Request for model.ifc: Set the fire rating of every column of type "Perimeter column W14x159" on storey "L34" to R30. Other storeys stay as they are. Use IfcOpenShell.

First a look at what the model holds.

```python
import ifcopenshell
import ifcopenshell.util.element

model = ifcopenshell.open("model.ifc")
print(model.schema)
storey = next(s for s in model.by_type("IfcBuildingStorey") if s.Name == "L34")
columns = [e for e in ifcopenshell.util.element.get_decomposition(storey) if e.is_a("IfcColumn")]
seen = {}
for e in columns:
    element_type = ifcopenshell.util.element.get_type(e)
    key = (element_type.Name if element_type != e and element_type else None, ifcopenshell.util.element.get_pset(e, "Pset_ColumnCommon", "FireRating"))
    seen[key] = seen.get(key, 0) + 1
for (name, value), count in sorted(seen.items(), key=str):
    print(count, "x", name, "|", value)
```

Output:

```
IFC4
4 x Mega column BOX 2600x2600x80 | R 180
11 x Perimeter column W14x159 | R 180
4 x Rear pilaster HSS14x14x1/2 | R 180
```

```python
import ifcopenshell
import ifcopenshell.api.pset
import ifcopenshell.util.element

model = ifcopenshell.open("model.ifc")

storey = next(s for s in model.by_type("IfcBuildingStorey") if s.Name == "L34")
columns = [e for e in ifcopenshell.util.element.get_decomposition(storey) if e.is_a("IfcColumn")]

count = 0
for e in columns:
    element_type = ifcopenshell.util.element.get_type(e)
    if element_type in (None, e) or element_type.Name != "Perimeter column W14x159":
        continue
    found = ifcopenshell.util.element.get_pset(e, "Pset_ColumnCommon", should_inherit=False)
    if found:
        pset = model.by_id(found["id"])
        if len(ifcopenshell.util.element.get_elements_by_pset(pset)) > 1:
            pset = ifcopenshell.api.pset.unshare_pset(model, products=[e], pset=pset)[0]
    else:
        pset = ifcopenshell.api.pset.add_pset(model, product=e, name="Pset_ColumnCommon")
    ifcopenshell.api.pset.edit_pset(model, pset=pset, properties={"FireRating": "R30"})
    count += 1

print(count, "columns updated")

model.write("model_rev.ifc")
```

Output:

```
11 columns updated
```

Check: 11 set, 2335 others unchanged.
